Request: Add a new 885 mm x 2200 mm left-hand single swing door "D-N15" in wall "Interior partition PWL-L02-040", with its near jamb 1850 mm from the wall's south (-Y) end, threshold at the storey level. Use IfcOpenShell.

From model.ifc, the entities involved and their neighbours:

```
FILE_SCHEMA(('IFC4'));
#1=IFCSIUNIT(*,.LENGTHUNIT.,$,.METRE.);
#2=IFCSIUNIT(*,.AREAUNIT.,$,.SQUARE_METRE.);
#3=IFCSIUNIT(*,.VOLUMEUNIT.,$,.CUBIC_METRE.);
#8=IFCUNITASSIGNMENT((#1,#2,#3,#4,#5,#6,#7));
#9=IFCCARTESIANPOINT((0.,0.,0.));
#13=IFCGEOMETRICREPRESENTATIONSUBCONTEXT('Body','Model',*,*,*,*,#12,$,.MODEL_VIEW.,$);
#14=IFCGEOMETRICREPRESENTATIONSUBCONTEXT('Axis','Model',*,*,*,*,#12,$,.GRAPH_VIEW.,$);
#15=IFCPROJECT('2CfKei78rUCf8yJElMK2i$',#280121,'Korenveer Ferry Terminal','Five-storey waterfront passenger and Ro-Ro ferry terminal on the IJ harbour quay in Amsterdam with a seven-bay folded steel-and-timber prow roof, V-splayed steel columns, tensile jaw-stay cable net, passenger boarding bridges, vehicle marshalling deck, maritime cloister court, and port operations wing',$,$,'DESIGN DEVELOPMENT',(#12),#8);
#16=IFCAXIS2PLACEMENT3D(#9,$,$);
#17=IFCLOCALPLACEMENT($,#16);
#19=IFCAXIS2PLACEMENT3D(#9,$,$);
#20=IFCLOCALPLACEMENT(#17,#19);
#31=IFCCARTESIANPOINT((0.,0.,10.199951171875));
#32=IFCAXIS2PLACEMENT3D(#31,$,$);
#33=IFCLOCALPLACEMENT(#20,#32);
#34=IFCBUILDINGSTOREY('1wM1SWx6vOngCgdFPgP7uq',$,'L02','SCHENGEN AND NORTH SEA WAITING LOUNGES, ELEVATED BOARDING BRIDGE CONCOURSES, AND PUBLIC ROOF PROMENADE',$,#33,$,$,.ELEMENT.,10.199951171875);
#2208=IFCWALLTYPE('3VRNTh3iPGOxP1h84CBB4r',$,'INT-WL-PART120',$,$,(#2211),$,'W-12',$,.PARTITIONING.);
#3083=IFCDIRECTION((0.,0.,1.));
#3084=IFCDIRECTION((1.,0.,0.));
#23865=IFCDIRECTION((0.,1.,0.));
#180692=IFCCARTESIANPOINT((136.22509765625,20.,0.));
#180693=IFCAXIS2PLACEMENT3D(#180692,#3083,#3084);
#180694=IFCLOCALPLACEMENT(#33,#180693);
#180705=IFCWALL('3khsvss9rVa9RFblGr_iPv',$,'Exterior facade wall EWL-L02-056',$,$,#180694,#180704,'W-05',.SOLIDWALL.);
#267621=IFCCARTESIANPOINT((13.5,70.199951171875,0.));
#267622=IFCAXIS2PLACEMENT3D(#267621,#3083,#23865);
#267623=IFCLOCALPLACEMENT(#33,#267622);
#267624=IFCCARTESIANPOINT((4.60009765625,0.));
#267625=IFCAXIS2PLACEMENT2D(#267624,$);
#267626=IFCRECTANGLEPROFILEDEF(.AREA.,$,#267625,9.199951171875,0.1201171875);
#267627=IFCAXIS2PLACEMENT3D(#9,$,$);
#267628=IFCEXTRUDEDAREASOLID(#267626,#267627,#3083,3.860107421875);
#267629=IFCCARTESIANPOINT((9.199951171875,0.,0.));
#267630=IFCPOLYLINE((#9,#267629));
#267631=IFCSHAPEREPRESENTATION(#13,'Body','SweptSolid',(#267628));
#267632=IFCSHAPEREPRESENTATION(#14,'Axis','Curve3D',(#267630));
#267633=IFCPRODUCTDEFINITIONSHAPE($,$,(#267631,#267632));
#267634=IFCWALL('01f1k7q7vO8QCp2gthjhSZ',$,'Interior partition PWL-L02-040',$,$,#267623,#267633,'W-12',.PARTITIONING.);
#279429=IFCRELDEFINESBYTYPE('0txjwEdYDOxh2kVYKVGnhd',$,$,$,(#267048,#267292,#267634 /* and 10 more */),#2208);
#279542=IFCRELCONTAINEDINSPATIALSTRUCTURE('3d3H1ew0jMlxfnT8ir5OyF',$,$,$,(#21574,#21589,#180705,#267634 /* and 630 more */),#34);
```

```python
import numpy as np
import ifcopenshell
import ifcopenshell.api.feature
import ifcopenshell.api.geometry
import ifcopenshell.api.root
import ifcopenshell.api.spatial
import ifcopenshell.geom
import ifcopenshell.util.element
import ifcopenshell.util.placement
import ifcopenshell.util.representation
import ifcopenshell.util.shape
import ifcopenshell.util.unit

model = ifcopenshell.open("model.ifc")
unit_scale = ifcopenshell.util.unit.calculate_unit_scale(model)
settings = ifcopenshell.geom.settings()


def volume(element):
    """Net volume in cubic metres, openings subtracted."""
    shape = ifcopenshell.geom.create_shape(settings, element)
    return ifcopenshell.util.shape.get_volume(shape.geometry)


wall = model.by_id(267634)
storey = ifcopenshell.util.element.get_container(wall, ifc_class="IfcBuildingStorey")
context = ifcopenshell.util.representation.get_context(model, "Model", "Body", "MODEL_VIEW")
before = volume(wall)

width, height, from_end, sill = 0.885, 2.2, 1.85, 0.0  # metres

# The wall runs along its own X axis, and the end named is its -X end.
wall_shape = ifcopenshell.geom.create_shape(settings, wall)
x, y, z = ifcopenshell.util.shape.get_vertices(wall_shape.geometry).T
start = x.min() + from_end
face, thickness = float(y.min()), float(y.max() - y.min())
wall_matrix = ifcopenshell.util.placement.get_local_placement(wall.ObjectPlacement)
level = ifcopenshell.util.placement.get_local_placement(storey.ObjectPlacement)[2, 3]


def in_wall(x, y):
    """Placement at x, y metres in the wall's axes, at sill height."""
    matrix = wall_matrix.copy()
    matrix[:, 3] = wall_matrix @ np.array([x / unit_scale, y / unit_scale, 0.0, 1.0])
    matrix[2, 3] = level + sill / unit_scale
    return matrix


# Opening: a box that overshoots both wall faces by 50 mm.
opening = ifcopenshell.api.root.create_entity(model, ifc_class="IfcOpeningElement", predefined_type="OPENING")
box = ifcopenshell.api.geometry.add_wall_representation(
    model, context=context, length=width, height=height, thickness=thickness + 0.1
)
ifcopenshell.api.geometry.assign_representation(model, product=opening, representation=box)
ifcopenshell.api.geometry.edit_object_placement(model, product=opening, matrix=in_wall(start, face - 0.05), is_si=False)
ifcopenshell.api.feature.add_feature(model, feature=opening, element=wall)

door = ifcopenshell.api.root.create_entity(model, ifc_class="IfcDoor", name="D-N15", predefined_type="DOOR")
door.OverallWidth, door.OverallHeight = width / unit_scale, height / unit_scale
door.OperationType = "SINGLE_SWING_LEFT"
body = ifcopenshell.api.geometry.add_door_representation(
    model,
    context=context,
    overall_width=door.OverallWidth,
    overall_height=door.OverallHeight,
    operation_type="SINGLE_SWING_LEFT",
    lining_properties={"LiningDepth": thickness / unit_scale, "ThresholdDepth": thickness / unit_scale},
)
ifcopenshell.api.geometry.assign_representation(model, product=door, representation=body)
ifcopenshell.api.spatial.assign_container(model, products=[door], relating_structure=storey)
ifcopenshell.api.feature.add_filling(model, opening=opening, element=door)

# The lining spans the wall, so the door starts at the wall face.
ifcopenshell.api.geometry.edit_object_placement(model, product=door, matrix=in_wall(start, face), is_si=False)

after = volume(wall)

print(f"wall volume {before:.3f} -> {after:.3f} m3")

model.write("model_v2.ifc")
```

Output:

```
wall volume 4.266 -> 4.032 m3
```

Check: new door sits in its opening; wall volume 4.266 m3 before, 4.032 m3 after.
